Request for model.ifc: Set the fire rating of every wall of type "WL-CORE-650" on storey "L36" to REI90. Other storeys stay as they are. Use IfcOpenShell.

First a look at what the model holds.

```python
import ifcopenshell
import ifcopenshell.util.element

model = ifcopenshell.open("model.ifc")
print(model.schema)
storey = next(s for s in model.by_type("IfcBuildingStorey") if s.Name == "L36")
walls = [e for e in ifcopenshell.util.element.get_decomposition(storey) if e.is_a("IfcWall")]
seen = {}
for e in walls:
    element_type = ifcopenshell.util.element.get_type(e)
    key = (element_type.Name if element_type != e and element_type else None, ifcopenshell.util.element.get_pset(e, "Pset_WallCommon", "FireRating"))
    seen[key] = seen.get(key, 0) + 1
for (name, value), count in sorted(seen.items(), key=str):
    print(count, "x", name, "|", value)
```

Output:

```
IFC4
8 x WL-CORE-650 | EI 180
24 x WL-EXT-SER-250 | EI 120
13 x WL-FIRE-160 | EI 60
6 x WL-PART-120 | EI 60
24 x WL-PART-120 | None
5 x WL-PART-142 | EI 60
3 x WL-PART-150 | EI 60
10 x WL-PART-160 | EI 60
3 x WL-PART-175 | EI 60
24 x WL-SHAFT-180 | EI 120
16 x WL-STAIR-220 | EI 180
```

```python
import ifcopenshell
import ifcopenshell.api.pset
import ifcopenshell.util.element

model = ifcopenshell.open("model.ifc")

storey = next(s for s in model.by_type("IfcBuildingStorey") if s.Name == "L36")
walls = [e for e in ifcopenshell.util.element.get_decomposition(storey) if e.is_a("IfcWall")]

count = 0
for e in walls:
    element_type = ifcopenshell.util.element.get_type(e)
    if element_type in (None, e) or element_type.Name != "WL-CORE-650":
        continue
    found = ifcopenshell.util.element.get_pset(e, "Pset_WallCommon", should_inherit=False)
    if found:
        pset = model.by_id(found["id"])
        if len(ifcopenshell.util.element.get_elements_by_pset(pset)) > 1:
            pset = ifcopenshell.api.pset.unshare_pset(model, products=[e], pset=pset)[0]
    else:
        pset = ifcopenshell.api.pset.add_pset(model, product=e, name="Pset_WallCommon")
    ifcopenshell.api.pset.edit_pset(model, pset=pset, properties={"FireRating": "REI90"})
    count += 1

print(count, "walls updated")

model.write("model-out.ifc")
```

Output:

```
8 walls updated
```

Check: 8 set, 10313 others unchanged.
